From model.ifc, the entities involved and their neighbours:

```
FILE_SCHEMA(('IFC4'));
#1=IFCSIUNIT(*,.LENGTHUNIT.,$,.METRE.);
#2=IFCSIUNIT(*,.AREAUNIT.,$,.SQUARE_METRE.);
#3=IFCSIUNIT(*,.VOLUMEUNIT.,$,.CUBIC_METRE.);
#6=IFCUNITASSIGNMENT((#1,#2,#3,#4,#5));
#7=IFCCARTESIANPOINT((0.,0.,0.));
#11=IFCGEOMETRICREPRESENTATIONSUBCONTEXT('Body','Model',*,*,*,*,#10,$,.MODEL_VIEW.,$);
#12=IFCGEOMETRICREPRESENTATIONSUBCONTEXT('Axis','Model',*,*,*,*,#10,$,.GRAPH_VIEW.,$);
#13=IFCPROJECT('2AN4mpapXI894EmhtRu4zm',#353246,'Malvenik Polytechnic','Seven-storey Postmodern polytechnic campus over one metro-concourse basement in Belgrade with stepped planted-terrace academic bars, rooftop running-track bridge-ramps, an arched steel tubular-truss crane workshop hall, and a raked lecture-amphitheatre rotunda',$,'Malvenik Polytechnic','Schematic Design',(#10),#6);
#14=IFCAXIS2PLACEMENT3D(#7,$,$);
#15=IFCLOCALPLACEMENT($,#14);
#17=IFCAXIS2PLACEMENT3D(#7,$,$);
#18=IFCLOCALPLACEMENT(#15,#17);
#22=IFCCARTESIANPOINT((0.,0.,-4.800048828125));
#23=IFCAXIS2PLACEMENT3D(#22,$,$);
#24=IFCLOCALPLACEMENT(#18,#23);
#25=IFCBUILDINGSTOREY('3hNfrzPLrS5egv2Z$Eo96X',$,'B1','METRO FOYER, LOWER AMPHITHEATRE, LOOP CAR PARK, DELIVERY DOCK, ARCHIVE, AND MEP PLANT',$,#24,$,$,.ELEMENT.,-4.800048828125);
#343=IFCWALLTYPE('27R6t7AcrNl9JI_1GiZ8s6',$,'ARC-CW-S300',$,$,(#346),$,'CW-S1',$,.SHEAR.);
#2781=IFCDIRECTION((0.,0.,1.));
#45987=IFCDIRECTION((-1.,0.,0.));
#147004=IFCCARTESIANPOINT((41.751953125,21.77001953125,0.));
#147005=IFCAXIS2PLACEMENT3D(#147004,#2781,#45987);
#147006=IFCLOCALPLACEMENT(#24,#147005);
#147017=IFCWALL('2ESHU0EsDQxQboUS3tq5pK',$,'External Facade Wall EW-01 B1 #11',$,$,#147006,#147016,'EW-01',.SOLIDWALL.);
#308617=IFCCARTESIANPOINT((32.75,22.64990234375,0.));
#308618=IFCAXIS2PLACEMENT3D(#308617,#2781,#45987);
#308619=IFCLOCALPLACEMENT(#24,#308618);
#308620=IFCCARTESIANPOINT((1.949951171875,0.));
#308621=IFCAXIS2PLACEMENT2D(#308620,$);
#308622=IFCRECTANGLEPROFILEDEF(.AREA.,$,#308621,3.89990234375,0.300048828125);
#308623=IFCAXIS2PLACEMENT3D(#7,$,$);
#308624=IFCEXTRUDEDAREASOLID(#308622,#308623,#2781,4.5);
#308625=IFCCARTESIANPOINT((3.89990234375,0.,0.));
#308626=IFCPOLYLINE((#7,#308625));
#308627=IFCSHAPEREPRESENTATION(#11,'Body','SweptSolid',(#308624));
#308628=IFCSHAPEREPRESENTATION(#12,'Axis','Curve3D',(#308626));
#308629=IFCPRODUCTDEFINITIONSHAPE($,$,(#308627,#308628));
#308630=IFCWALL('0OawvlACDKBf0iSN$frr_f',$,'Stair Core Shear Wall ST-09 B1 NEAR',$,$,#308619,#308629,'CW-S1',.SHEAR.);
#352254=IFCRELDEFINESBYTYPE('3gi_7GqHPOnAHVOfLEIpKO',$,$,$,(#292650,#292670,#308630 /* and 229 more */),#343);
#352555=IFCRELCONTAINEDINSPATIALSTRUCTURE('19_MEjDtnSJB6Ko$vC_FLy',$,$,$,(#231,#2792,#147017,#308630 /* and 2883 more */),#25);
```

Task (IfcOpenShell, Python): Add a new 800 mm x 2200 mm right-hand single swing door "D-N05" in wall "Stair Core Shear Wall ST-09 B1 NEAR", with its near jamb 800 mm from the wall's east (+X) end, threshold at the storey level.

```python
import numpy as np
import ifcopenshell
import ifcopenshell.api.feature
import ifcopenshell.api.geometry
import ifcopenshell.api.root
import ifcopenshell.api.spatial
import ifcopenshell.geom
import ifcopenshell.util.element
import ifcopenshell.util.placement
import ifcopenshell.util.representation
import ifcopenshell.util.shape
import ifcopenshell.util.unit

model = ifcopenshell.open("model.ifc")
unit_scale = ifcopenshell.util.unit.calculate_unit_scale(model)
settings = ifcopenshell.geom.settings()


def volume(element):
    """Net volume in cubic metres, openings subtracted."""
    shape = ifcopenshell.geom.create_shape(settings, element)
    return ifcopenshell.util.shape.get_volume(shape.geometry)


wall = model.by_guid("0OawvlACDKBf0iSN$frr_f")
storey = ifcopenshell.util.element.get_container(wall, ifc_class="IfcBuildingStorey")
context = ifcopenshell.util.representation.get_context(model, "Model", "Body", "MODEL_VIEW")
before = volume(wall)

width, height, from_end, sill = 0.8, 2.2, 0.8, 0.0  # metres

# The wall runs along its own X axis, and the end named is its -X end.
wall_shape = ifcopenshell.geom.create_shape(settings, wall)
x, y, z = ifcopenshell.util.shape.get_vertices(wall_shape.geometry).T
start = x.min() + from_end
face, thickness = float(y.min()), float(y.max() - y.min())
wall_matrix = ifcopenshell.util.placement.get_local_placement(wall.ObjectPlacement)
level = ifcopenshell.util.placement.get_local_placement(storey.ObjectPlacement)[2, 3]


def in_wall(x, y):
    """Placement at x, y metres in the wall's axes, at sill height."""
    matrix = wall_matrix.copy()
    matrix[:, 3] = wall_matrix @ np.array([x / unit_scale, y / unit_scale, 0.0, 1.0])
    matrix[2, 3] = level + sill / unit_scale
    return matrix


# Opening: a box that overshoots both wall faces by 50 mm.
opening = ifcopenshell.api.root.create_entity(model, ifc_class="IfcOpeningElement", predefined_type="OPENING")
box = ifcopenshell.api.geometry.add_wall_representation(
    model, context=context, length=width, height=height, thickness=thickness + 0.1
)
ifcopenshell.api.geometry.assign_representation(model, product=opening, representation=box)
ifcopenshell.api.geometry.edit_object_placement(model, product=opening, matrix=in_wall(start, face - 0.05), is_si=False)
ifcopenshell.api.feature.add_feature(model, feature=opening, element=wall)

door = ifcopenshell.api.root.create_entity(model, ifc_class="IfcDoor", name="D-N05", predefined_type="DOOR")
door.OverallWidth, door.OverallHeight = width / unit_scale, height / unit_scale
door.OperationType = "SINGLE_SWING_RIGHT"
body = ifcopenshell.api.geometry.add_door_representation(
    model,
    context=context,
    overall_width=door.OverallWidth,
    overall_height=door.OverallHeight,
    operation_type="SINGLE_SWING_RIGHT",
    lining_properties={"LiningDepth": thickness / unit_scale, "ThresholdDepth": thickness / unit_scale},
)
ifcopenshell.api.geometry.assign_representation(model, product=door, representation=body)
ifcopenshell.api.spatial.assign_container(model, products=[door], relating_structure=storey)
ifcopenshell.api.feature.add_filling(model, opening=opening, element=door)

# The lining spans the wall, so the door starts at the wall face.
ifcopenshell.api.geometry.edit_object_placement(model, product=door, matrix=in_wall(start, face), is_si=False)

after = volume(wall)

print(f"wall volume {before:.3f} -> {after:.3f} m3")

model.write("model_edited.ifc")
```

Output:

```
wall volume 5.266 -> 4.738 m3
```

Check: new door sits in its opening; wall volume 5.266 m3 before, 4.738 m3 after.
